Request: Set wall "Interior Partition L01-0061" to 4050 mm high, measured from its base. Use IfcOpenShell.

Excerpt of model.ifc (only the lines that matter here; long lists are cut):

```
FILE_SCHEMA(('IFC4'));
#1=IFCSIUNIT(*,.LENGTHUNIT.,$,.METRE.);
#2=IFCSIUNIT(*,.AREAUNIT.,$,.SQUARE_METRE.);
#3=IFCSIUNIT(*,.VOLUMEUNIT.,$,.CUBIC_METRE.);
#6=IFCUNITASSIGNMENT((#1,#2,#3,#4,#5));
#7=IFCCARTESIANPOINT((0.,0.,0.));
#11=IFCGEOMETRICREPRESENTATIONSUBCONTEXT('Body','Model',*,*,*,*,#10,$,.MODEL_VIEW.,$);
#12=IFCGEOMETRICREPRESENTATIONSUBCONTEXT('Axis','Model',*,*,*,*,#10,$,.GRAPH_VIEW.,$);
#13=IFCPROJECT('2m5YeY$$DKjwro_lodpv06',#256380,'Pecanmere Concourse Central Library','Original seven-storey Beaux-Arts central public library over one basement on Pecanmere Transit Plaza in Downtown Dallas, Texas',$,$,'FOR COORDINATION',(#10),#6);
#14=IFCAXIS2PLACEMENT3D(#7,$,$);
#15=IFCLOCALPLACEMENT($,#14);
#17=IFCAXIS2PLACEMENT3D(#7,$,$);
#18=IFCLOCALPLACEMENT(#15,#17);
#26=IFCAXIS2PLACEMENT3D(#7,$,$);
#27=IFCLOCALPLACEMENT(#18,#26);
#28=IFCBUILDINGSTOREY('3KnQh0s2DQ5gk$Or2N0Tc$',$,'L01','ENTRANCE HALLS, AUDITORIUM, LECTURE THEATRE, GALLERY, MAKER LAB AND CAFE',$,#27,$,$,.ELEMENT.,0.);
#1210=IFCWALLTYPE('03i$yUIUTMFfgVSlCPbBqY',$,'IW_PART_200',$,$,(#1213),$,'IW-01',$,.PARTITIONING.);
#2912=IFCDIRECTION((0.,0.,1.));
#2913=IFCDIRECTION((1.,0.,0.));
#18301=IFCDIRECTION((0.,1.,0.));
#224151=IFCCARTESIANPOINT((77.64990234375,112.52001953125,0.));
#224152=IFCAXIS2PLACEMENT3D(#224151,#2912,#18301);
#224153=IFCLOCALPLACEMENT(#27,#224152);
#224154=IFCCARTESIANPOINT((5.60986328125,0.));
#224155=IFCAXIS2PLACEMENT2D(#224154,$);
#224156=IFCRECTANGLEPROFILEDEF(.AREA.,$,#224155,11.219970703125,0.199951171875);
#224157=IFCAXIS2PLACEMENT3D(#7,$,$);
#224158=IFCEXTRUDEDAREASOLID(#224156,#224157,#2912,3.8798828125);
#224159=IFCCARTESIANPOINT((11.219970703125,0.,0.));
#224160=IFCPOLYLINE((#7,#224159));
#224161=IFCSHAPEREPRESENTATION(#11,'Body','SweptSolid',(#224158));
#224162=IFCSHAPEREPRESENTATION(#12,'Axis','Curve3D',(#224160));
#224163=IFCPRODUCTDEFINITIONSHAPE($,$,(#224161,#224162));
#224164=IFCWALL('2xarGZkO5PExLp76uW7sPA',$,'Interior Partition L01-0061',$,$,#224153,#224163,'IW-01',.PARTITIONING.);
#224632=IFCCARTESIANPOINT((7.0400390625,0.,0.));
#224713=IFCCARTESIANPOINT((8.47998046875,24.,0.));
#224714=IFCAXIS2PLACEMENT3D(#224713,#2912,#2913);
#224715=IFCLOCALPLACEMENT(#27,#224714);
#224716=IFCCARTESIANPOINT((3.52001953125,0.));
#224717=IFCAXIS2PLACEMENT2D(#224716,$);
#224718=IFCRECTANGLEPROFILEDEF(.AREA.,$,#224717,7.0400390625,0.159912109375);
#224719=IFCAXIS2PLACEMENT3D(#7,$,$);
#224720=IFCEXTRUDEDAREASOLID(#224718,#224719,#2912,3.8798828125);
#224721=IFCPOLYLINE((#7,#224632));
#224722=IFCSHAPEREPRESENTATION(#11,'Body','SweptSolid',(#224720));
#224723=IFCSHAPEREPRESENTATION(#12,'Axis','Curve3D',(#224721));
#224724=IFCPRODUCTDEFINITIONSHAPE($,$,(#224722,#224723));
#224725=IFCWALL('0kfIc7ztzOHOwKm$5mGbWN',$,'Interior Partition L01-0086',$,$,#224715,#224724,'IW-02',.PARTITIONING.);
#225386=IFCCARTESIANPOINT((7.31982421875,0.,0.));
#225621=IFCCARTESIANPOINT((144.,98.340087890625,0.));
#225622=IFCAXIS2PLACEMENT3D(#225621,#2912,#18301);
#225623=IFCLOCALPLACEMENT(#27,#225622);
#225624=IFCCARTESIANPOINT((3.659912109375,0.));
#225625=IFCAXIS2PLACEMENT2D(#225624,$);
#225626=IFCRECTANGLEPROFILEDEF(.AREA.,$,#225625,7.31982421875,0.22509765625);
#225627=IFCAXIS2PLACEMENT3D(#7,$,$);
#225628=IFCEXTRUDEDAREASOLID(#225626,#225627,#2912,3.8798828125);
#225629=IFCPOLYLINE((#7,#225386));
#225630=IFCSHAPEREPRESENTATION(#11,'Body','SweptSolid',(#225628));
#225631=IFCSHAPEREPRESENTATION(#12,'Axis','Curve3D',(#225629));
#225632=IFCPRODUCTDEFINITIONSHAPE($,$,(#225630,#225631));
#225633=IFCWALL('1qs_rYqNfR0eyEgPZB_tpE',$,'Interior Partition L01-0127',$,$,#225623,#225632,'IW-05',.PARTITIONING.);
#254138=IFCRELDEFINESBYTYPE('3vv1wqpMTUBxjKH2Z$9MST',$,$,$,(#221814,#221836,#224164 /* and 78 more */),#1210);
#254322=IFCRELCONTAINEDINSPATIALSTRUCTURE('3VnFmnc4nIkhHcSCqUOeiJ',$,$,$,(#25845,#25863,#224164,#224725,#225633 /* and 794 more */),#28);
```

```python
import ifcopenshell
import ifcopenshell.geom
import ifcopenshell.util.representation
import ifcopenshell.util.shape

model = ifcopenshell.open("model.ifc")
settings = ifcopenshell.geom.settings()


def volume(element):
    """Net volume in cubic metres, openings subtracted."""
    shape = ifcopenshell.geom.create_shape(settings, element)
    return ifcopenshell.util.shape.get_volume(shape.geometry)


wall = model.by_guid("2xarGZkO5PExLp76uW7sPA")
before = volume(wall)

body = ifcopenshell.util.representation.get_representation(wall, "Model", "Body")
solid = body.Items[0]
old_height = solid.Depth
solid.Depth = 4.05
after = volume(wall)

print(f"height {old_height:g} -> {solid.Depth:g}, volume {before:.3f} -> {after:.3f} m3")

model.write("model_edited.ifc")
```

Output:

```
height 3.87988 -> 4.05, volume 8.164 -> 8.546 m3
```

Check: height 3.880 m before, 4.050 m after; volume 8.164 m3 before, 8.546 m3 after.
